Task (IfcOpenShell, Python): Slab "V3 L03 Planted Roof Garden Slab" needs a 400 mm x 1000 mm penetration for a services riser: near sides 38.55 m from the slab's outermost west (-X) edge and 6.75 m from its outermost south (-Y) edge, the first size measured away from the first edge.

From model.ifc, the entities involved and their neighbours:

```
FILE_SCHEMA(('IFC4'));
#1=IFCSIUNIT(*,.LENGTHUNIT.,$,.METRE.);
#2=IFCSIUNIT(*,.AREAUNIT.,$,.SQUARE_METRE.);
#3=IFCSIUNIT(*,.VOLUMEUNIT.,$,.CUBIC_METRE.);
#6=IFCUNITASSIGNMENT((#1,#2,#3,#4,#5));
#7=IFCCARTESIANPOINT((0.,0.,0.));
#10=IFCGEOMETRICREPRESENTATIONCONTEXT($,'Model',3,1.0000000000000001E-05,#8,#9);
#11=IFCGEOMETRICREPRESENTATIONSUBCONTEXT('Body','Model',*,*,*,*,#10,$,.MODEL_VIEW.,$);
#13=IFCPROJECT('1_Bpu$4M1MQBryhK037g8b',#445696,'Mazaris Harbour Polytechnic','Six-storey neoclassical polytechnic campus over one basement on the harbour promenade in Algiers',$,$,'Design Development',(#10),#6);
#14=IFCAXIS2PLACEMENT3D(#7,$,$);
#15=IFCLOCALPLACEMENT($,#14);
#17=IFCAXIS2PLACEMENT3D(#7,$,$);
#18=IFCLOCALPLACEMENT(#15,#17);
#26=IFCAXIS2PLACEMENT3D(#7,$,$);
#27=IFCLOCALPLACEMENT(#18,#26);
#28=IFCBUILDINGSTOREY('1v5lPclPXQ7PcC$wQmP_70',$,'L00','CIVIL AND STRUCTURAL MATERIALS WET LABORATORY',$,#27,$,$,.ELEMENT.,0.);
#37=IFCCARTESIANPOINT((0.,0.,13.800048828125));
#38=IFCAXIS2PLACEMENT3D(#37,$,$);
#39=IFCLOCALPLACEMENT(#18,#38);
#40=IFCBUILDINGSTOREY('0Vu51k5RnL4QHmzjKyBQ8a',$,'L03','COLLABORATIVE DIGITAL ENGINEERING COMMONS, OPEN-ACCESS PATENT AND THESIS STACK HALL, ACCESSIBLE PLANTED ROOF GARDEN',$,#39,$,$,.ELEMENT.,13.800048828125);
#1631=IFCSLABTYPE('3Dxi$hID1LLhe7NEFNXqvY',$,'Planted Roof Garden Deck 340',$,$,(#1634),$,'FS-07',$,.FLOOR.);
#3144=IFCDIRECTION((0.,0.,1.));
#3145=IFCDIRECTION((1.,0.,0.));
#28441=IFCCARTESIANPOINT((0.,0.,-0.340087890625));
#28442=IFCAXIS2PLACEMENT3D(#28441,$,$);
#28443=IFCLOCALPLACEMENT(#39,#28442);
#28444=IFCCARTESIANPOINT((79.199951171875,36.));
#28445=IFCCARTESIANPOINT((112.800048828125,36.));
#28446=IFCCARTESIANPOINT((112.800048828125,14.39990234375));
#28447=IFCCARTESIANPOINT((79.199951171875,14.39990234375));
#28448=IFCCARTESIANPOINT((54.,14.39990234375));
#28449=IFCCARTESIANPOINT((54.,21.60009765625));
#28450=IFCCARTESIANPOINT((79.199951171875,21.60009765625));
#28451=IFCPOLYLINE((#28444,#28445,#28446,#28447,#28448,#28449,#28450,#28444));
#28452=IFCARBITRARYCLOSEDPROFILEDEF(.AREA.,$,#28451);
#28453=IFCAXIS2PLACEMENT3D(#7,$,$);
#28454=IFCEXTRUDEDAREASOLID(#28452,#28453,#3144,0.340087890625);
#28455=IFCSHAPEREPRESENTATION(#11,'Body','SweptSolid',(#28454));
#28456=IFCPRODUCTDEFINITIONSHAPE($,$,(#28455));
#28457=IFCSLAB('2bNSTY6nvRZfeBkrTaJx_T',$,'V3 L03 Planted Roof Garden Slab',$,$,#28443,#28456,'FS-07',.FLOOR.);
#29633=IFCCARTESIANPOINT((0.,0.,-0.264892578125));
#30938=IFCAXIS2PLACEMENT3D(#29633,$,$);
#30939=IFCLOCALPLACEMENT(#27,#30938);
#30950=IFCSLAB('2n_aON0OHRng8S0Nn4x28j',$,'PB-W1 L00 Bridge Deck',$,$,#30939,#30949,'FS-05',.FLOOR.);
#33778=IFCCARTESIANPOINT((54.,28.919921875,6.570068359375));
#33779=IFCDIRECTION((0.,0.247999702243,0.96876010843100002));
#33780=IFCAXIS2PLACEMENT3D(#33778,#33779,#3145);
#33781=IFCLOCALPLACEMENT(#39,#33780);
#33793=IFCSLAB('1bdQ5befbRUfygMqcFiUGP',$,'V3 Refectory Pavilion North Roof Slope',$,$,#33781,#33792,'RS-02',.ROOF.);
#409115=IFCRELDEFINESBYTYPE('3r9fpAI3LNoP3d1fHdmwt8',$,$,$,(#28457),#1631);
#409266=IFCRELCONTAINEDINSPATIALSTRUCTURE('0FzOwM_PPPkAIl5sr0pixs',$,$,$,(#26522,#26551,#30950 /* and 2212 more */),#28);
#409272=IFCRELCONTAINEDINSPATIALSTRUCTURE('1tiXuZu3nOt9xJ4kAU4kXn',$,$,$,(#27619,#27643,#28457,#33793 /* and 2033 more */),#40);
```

```python
import numpy as np
import ifcopenshell
import ifcopenshell.api.feature
import ifcopenshell.api.geometry
import ifcopenshell.api.root
import ifcopenshell.geom
import ifcopenshell.util.placement
import ifcopenshell.util.representation
import ifcopenshell.util.shape
import ifcopenshell.util.unit

model = ifcopenshell.open("model.ifc")
unit_scale = ifcopenshell.util.unit.calculate_unit_scale(model)
settings = ifcopenshell.geom.settings()


def volume(element):
    """Net volume in cubic metres, openings subtracted."""
    shape = ifcopenshell.geom.create_shape(settings, element)
    return ifcopenshell.util.shape.get_volume(shape.geometry)


slab = model.by_guid("2bNSTY6nvRZfeBkrTaJx_T")
before = volume(slab)

# Extent in the slab's own axes, in metres. The edges named are its -X and -Y sides.
slab_shape = ifcopenshell.geom.create_shape(settings, slab)
vertices = ifcopenshell.util.shape.get_vertices(slab_shape.geometry)
x_min, y_min, bottom = vertices.min(axis=0)
top = vertices[:, 2].max()

opening = ifcopenshell.api.root.create_entity(model, ifc_class="IfcOpeningElement", name="Services riser opening", predefined_type="OPENING")
context = ifcopenshell.util.representation.get_context(model, "Model", "Body", "MODEL_VIEW")
width, depth = 0.4, 1
outline = [(0.0, 0.0), (width, 0.0), (width, depth), (0.0, depth), (0.0, 0.0)]
# Overshoot both faces by 50 mm so the cut is clean.
shape = ifcopenshell.api.geometry.add_slab_representation(
    model, context=context, depth=top - bottom + 0.1, polyline=outline
)
ifcopenshell.api.geometry.assign_representation(model, product=opening, representation=shape)

matrix = ifcopenshell.util.placement.get_local_placement(slab.ObjectPlacement)
matrix[:, 3] = matrix @ np.append(np.array([x_min + 38.55, y_min + 6.75, bottom - 0.05]) / unit_scale, 1.0)
ifcopenshell.api.geometry.edit_object_placement(model, product=opening, matrix=matrix, is_si=False)
ifcopenshell.api.feature.add_feature(model, feature=opening, element=slab)

after = volume(slab)

print(f"slab volume {before:.3f} -> {after:.3f} m3")

model.write("model_updated.ifc")
```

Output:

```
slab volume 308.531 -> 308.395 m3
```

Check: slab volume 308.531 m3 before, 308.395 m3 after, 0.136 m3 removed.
